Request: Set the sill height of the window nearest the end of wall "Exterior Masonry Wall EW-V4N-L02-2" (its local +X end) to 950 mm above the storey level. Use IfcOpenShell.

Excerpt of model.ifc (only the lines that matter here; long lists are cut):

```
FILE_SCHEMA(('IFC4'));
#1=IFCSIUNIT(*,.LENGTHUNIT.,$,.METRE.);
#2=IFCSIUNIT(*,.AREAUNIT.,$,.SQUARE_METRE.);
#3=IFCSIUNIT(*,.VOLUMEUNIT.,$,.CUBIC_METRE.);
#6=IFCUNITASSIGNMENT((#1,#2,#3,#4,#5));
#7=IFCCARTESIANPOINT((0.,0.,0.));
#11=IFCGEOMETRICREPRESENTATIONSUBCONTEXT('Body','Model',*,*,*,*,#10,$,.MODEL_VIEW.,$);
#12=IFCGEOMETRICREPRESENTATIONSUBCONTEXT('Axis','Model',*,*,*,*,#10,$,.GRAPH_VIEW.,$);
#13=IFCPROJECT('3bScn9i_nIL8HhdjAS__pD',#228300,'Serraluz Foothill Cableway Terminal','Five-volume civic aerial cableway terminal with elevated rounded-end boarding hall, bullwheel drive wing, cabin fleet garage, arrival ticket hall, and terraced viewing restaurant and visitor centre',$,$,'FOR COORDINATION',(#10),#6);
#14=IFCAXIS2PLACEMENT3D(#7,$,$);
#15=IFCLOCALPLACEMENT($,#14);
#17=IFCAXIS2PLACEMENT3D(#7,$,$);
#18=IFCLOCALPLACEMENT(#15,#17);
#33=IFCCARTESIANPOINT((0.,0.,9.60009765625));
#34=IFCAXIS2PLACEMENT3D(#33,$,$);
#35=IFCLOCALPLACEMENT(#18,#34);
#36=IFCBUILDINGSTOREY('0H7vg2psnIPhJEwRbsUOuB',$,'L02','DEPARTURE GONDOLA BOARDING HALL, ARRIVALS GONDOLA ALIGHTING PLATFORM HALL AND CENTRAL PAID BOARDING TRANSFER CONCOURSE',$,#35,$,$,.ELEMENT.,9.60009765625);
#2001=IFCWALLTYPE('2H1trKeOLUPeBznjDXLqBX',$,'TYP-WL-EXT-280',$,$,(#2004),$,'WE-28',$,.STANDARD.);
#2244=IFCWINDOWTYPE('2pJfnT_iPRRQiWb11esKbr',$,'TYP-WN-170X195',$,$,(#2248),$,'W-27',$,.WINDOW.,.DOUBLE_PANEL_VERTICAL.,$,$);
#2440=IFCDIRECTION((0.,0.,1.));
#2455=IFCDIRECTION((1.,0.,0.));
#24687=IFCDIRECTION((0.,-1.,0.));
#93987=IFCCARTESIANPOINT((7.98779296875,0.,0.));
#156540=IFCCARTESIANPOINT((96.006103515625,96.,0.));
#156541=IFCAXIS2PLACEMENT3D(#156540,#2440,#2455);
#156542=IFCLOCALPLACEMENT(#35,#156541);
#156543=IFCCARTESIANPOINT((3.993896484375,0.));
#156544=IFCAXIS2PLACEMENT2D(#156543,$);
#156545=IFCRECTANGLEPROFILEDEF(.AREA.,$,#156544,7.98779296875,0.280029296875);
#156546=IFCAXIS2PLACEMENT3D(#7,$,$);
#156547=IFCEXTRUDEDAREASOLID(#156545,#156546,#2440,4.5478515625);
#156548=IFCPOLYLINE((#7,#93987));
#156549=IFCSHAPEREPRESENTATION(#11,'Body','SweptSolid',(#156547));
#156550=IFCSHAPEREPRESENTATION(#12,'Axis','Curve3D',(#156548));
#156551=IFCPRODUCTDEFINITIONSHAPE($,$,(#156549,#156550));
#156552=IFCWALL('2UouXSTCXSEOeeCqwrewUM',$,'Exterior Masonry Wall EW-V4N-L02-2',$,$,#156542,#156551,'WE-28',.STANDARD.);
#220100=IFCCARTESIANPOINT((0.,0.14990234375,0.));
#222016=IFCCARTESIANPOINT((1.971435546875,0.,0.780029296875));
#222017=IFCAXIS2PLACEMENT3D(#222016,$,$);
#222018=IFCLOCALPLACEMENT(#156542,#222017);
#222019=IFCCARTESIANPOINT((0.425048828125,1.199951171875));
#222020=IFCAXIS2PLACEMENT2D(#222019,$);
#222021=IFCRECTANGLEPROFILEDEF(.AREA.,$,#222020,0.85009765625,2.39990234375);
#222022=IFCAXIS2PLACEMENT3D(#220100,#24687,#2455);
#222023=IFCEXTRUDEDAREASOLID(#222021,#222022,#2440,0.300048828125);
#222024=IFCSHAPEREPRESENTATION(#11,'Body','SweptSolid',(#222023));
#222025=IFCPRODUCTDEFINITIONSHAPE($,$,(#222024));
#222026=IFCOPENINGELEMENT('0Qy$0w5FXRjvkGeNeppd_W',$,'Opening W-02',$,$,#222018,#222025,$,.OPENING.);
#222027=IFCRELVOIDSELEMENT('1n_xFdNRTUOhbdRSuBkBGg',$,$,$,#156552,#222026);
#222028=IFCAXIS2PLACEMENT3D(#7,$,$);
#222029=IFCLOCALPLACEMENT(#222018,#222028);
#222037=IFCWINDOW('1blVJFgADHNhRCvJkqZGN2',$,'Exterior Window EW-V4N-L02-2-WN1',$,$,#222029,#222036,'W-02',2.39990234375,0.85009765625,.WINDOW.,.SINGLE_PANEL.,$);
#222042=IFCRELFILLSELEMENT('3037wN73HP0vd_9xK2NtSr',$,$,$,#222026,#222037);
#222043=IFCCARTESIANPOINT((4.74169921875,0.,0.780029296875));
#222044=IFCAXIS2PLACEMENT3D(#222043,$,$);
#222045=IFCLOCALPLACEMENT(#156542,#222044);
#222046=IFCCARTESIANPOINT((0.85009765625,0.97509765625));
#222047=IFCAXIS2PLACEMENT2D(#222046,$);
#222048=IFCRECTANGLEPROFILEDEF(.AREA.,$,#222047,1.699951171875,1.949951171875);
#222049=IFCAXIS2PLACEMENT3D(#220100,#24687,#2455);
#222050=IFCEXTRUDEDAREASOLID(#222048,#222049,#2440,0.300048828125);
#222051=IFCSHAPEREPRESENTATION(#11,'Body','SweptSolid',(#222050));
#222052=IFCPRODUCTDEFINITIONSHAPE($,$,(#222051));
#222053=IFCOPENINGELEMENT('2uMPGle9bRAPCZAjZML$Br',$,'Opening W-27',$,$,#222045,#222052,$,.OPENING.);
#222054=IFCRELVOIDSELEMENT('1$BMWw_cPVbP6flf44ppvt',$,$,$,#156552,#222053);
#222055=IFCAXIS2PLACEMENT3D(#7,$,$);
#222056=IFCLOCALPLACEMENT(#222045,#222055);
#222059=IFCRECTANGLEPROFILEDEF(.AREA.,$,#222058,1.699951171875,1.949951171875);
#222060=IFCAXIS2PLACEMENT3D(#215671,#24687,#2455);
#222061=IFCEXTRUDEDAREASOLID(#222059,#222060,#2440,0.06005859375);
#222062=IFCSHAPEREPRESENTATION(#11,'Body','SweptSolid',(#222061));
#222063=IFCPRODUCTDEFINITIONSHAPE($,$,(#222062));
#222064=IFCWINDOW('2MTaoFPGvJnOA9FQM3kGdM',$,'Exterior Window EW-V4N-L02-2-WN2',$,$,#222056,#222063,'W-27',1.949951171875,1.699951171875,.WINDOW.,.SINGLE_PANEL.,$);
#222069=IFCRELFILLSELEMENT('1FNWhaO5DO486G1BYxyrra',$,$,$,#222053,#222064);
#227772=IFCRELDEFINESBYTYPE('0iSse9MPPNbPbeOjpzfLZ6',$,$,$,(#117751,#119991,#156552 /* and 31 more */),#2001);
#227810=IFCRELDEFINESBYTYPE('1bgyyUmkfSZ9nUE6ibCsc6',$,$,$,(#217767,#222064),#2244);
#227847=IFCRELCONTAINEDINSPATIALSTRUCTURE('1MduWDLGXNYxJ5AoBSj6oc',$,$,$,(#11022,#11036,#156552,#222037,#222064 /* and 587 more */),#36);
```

```python
import numpy as np
import ifcopenshell
import ifcopenshell.api.geometry
import ifcopenshell.geom
import ifcopenshell.util.element
import ifcopenshell.util.placement
import ifcopenshell.util.shape
import ifcopenshell.util.unit

model = ifcopenshell.open("model.ifc")
unit_scale = ifcopenshell.util.unit.calculate_unit_scale(model)

window = model.by_guid("2MTaoFPGvJnOA9FQM3kGdM")
opening = window.FillsVoids[0].RelatingOpeningElement
storey = ifcopenshell.util.element.get_container(window, ifc_class="IfcBuildingStorey")
level = ifcopenshell.util.placement.get_local_placement(storey.ObjectPlacement)[2, 3]

# The opening's origin need not be at the sill, so measure its lowest point.
shape = ifcopenshell.geom.create_shape(ifcopenshell.geom.settings(), opening)
bottom = ifcopenshell.util.shape.get_shape_bottom_elevation(shape, shape.geometry) / unit_scale
dz = level + 0.95 - bottom

shift = np.array([0.0, 0.0, dz])
# The window is placed relative to its opening, so it follows when the opening moves.
matrix = ifcopenshell.util.placement.get_local_placement(opening.ObjectPlacement)
matrix[:3, 3] += shift
ifcopenshell.api.geometry.edit_object_placement(
    model, product=opening, matrix=matrix, is_si=False, should_transform_children=True
)

print(f"moved by {dz * unit_scale:+.3f} m")

model.write("model_updated.ifc")
```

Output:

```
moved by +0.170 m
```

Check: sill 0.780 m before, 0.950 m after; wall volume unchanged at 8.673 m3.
